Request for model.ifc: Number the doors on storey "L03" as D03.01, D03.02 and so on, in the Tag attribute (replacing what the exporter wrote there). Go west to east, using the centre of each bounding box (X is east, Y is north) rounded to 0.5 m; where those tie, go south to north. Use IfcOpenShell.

First a look at what the model holds.

```python
import ifcopenshell
import ifcopenshell.util.element
import ifcopenshell.util.placement

model = ifcopenshell.open("model.ifc")
print(model.schema)
storey = next(s for s in model.by_type("IfcBuildingStorey") if s.Name == "L03")
doors = [e for e in ifcopenshell.util.element.get_decomposition(storey) if e.is_a("IfcDoor")]
for e in sorted(doors, key=lambda e: e.id()):
    origin = ifcopenshell.util.placement.get_local_placement(e.ObjectPlacement)[:3, 3]
    print(e.id(), e.Tag, e.Name, origin.round(2) + 0.0, sep=" | ")
```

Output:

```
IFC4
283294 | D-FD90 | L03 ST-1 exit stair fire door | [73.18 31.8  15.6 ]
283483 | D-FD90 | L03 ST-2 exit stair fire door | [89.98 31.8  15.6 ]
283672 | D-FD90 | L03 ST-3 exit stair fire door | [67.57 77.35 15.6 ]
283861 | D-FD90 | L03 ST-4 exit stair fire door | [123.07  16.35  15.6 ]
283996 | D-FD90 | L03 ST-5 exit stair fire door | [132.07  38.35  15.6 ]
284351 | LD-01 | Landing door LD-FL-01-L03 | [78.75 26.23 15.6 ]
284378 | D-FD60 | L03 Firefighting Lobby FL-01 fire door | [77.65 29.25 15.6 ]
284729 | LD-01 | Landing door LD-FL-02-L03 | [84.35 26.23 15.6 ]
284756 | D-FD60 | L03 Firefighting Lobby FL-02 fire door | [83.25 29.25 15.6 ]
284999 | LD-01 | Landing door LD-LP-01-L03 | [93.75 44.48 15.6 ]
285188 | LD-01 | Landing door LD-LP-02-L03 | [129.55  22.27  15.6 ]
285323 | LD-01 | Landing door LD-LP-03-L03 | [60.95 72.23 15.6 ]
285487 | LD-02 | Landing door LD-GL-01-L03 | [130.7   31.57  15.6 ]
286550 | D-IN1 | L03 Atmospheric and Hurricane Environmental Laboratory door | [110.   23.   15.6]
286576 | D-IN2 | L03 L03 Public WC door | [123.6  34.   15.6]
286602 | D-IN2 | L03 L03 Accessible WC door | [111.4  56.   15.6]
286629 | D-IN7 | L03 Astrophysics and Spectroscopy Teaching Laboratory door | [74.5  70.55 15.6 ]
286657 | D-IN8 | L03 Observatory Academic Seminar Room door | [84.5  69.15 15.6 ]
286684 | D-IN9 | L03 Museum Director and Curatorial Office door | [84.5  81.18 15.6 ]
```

```python
import ifcopenshell
import ifcopenshell.geom
import ifcopenshell.util.element
import ifcopenshell.util.shape

model = ifcopenshell.open("model.ifc")
settings = ifcopenshell.geom.settings()
settings.set("use-world-coords", True)


def centre(element):
    shape = ifcopenshell.geom.create_shape(settings, element)
    return ifcopenshell.util.shape.get_bbox_centroid(shape.geometry)


storey = next(s for s in model.by_type("IfcBuildingStorey") if s.Name == "L03")
doors = [e for e in ifcopenshell.util.element.get_decomposition(storey) if e.is_a("IfcDoor")]

# Insertion points can sit at a corner or the storey origin, so sort by the geometry (in metres).
centres = {e: centre(e) for e in doors}
doors.sort(key=lambda e: (round(centres[e][0] / 0.5), centres[e][1]))

for i, e in enumerate(doors, start=1):
    number = f"D03.{i:02d}"
    e.Tag = number
    print(e.id(), number)

model.write("model_updated.ifc")
```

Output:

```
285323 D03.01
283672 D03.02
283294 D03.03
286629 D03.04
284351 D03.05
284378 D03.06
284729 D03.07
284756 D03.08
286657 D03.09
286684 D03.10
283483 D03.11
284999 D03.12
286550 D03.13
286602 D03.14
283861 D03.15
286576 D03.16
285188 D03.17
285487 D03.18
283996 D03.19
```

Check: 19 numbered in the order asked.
